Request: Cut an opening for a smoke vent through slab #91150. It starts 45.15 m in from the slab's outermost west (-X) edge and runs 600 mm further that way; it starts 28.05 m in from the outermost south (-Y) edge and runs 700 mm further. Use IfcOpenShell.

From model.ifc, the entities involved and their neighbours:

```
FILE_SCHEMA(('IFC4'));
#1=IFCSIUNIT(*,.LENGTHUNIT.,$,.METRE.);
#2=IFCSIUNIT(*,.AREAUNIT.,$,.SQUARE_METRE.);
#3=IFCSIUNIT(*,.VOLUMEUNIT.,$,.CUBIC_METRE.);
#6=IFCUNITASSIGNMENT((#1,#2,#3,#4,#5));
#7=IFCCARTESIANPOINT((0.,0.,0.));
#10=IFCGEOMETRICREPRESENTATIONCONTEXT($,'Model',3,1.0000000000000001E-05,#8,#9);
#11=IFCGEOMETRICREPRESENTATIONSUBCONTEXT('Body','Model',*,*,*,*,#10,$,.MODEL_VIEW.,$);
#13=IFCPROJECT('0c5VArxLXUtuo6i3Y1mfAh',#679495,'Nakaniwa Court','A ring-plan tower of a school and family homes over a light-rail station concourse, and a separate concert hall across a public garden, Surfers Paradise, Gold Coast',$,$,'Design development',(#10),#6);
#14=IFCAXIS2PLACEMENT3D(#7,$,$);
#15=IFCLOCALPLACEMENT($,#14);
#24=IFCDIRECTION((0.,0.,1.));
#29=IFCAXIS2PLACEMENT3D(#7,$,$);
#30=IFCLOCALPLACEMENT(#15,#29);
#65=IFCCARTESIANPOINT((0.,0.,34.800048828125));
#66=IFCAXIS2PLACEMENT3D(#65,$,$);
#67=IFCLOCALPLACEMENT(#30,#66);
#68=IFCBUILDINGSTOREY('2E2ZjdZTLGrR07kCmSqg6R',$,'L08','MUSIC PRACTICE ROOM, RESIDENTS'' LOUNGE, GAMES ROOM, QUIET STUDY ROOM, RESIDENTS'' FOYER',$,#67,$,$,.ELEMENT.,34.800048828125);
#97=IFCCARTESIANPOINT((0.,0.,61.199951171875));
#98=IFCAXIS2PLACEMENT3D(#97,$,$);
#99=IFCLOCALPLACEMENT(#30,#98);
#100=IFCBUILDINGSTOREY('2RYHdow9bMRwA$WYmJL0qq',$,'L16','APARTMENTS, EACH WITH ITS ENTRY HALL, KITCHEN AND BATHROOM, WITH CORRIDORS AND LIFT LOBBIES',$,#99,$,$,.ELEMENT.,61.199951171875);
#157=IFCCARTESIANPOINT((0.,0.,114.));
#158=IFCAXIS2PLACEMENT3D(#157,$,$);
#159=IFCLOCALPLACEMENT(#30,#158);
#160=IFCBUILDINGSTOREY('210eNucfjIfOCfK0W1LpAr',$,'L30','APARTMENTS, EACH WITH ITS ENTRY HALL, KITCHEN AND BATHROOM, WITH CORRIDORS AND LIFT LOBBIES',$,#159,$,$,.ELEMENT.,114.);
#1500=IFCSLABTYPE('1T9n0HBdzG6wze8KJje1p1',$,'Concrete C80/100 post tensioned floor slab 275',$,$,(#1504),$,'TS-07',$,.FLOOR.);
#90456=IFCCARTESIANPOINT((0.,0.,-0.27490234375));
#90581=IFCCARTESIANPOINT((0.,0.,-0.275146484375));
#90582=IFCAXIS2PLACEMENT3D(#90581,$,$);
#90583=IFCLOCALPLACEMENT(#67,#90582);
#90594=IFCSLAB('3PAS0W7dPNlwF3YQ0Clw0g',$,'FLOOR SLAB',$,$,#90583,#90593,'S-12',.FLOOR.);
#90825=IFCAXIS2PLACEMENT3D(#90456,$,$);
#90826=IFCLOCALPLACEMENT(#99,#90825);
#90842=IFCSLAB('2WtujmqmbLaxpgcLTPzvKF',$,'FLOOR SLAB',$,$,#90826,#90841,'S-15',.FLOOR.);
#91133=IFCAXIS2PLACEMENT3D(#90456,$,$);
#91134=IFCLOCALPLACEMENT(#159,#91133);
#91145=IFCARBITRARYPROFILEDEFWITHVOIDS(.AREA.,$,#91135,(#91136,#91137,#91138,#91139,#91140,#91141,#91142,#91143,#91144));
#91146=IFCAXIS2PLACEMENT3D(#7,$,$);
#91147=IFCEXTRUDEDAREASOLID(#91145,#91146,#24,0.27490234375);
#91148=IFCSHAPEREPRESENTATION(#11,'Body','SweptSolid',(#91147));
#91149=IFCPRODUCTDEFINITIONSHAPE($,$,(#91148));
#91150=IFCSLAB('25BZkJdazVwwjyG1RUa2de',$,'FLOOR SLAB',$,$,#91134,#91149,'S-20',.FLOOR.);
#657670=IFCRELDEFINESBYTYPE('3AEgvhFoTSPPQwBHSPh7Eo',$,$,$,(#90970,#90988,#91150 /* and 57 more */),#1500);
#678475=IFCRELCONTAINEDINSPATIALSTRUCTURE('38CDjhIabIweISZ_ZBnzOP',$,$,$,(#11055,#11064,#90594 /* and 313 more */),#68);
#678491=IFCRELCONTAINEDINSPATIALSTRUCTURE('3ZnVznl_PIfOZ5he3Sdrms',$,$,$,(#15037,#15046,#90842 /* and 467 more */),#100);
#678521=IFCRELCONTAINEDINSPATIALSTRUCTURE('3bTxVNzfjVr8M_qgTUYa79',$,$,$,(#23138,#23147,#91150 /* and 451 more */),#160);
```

```python
import numpy as np
import ifcopenshell
import ifcopenshell.api.feature
import ifcopenshell.api.geometry
import ifcopenshell.api.root
import ifcopenshell.geom
import ifcopenshell.util.placement
import ifcopenshell.util.representation
import ifcopenshell.util.shape
import ifcopenshell.util.unit

model = ifcopenshell.open("model.ifc")
unit_scale = ifcopenshell.util.unit.calculate_unit_scale(model)
settings = ifcopenshell.geom.settings()


def volume(element):
    """Net volume in cubic metres, openings subtracted."""
    shape = ifcopenshell.geom.create_shape(settings, element)
    return ifcopenshell.util.shape.get_volume(shape.geometry)


slab = model.by_guid("25BZkJdazVwwjyG1RUa2de")
before = volume(slab)

# Extent in the slab's own axes, in metres. The edges named are its -X and -Y sides.
slab_shape = ifcopenshell.geom.create_shape(settings, slab)
vertices = ifcopenshell.util.shape.get_vertices(slab_shape.geometry)
x_min, y_min, bottom = vertices.min(axis=0)
top = vertices[:, 2].max()

opening = ifcopenshell.api.root.create_entity(model, ifc_class="IfcOpeningElement", name="Smoke vent opening", predefined_type="OPENING")
context = ifcopenshell.util.representation.get_context(model, "Model", "Body", "MODEL_VIEW")
width, depth = 0.6, 0.7
outline = [(0.0, 0.0), (width, 0.0), (width, depth), (0.0, depth), (0.0, 0.0)]
# Overshoot both faces by 50 mm so the cut is clean.
shape = ifcopenshell.api.geometry.add_slab_representation(
    model, context=context, depth=top - bottom + 0.1, polyline=outline
)
ifcopenshell.api.geometry.assign_representation(model, product=opening, representation=shape)

matrix = ifcopenshell.util.placement.get_local_placement(slab.ObjectPlacement)
matrix[:, 3] = matrix @ np.append(np.array([x_min + 45.15, y_min + 28.05, bottom - 0.05]) / unit_scale, 1.0)
ifcopenshell.api.geometry.edit_object_placement(model, product=opening, matrix=matrix, is_si=False)
ifcopenshell.api.feature.add_feature(model, feature=opening, element=slab)

after = volume(slab)

print(f"slab volume {before:.3f} -> {after:.3f} m3")

model.write("model_v2.ifc")
```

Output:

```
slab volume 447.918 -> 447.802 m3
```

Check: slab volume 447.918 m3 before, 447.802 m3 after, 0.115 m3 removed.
